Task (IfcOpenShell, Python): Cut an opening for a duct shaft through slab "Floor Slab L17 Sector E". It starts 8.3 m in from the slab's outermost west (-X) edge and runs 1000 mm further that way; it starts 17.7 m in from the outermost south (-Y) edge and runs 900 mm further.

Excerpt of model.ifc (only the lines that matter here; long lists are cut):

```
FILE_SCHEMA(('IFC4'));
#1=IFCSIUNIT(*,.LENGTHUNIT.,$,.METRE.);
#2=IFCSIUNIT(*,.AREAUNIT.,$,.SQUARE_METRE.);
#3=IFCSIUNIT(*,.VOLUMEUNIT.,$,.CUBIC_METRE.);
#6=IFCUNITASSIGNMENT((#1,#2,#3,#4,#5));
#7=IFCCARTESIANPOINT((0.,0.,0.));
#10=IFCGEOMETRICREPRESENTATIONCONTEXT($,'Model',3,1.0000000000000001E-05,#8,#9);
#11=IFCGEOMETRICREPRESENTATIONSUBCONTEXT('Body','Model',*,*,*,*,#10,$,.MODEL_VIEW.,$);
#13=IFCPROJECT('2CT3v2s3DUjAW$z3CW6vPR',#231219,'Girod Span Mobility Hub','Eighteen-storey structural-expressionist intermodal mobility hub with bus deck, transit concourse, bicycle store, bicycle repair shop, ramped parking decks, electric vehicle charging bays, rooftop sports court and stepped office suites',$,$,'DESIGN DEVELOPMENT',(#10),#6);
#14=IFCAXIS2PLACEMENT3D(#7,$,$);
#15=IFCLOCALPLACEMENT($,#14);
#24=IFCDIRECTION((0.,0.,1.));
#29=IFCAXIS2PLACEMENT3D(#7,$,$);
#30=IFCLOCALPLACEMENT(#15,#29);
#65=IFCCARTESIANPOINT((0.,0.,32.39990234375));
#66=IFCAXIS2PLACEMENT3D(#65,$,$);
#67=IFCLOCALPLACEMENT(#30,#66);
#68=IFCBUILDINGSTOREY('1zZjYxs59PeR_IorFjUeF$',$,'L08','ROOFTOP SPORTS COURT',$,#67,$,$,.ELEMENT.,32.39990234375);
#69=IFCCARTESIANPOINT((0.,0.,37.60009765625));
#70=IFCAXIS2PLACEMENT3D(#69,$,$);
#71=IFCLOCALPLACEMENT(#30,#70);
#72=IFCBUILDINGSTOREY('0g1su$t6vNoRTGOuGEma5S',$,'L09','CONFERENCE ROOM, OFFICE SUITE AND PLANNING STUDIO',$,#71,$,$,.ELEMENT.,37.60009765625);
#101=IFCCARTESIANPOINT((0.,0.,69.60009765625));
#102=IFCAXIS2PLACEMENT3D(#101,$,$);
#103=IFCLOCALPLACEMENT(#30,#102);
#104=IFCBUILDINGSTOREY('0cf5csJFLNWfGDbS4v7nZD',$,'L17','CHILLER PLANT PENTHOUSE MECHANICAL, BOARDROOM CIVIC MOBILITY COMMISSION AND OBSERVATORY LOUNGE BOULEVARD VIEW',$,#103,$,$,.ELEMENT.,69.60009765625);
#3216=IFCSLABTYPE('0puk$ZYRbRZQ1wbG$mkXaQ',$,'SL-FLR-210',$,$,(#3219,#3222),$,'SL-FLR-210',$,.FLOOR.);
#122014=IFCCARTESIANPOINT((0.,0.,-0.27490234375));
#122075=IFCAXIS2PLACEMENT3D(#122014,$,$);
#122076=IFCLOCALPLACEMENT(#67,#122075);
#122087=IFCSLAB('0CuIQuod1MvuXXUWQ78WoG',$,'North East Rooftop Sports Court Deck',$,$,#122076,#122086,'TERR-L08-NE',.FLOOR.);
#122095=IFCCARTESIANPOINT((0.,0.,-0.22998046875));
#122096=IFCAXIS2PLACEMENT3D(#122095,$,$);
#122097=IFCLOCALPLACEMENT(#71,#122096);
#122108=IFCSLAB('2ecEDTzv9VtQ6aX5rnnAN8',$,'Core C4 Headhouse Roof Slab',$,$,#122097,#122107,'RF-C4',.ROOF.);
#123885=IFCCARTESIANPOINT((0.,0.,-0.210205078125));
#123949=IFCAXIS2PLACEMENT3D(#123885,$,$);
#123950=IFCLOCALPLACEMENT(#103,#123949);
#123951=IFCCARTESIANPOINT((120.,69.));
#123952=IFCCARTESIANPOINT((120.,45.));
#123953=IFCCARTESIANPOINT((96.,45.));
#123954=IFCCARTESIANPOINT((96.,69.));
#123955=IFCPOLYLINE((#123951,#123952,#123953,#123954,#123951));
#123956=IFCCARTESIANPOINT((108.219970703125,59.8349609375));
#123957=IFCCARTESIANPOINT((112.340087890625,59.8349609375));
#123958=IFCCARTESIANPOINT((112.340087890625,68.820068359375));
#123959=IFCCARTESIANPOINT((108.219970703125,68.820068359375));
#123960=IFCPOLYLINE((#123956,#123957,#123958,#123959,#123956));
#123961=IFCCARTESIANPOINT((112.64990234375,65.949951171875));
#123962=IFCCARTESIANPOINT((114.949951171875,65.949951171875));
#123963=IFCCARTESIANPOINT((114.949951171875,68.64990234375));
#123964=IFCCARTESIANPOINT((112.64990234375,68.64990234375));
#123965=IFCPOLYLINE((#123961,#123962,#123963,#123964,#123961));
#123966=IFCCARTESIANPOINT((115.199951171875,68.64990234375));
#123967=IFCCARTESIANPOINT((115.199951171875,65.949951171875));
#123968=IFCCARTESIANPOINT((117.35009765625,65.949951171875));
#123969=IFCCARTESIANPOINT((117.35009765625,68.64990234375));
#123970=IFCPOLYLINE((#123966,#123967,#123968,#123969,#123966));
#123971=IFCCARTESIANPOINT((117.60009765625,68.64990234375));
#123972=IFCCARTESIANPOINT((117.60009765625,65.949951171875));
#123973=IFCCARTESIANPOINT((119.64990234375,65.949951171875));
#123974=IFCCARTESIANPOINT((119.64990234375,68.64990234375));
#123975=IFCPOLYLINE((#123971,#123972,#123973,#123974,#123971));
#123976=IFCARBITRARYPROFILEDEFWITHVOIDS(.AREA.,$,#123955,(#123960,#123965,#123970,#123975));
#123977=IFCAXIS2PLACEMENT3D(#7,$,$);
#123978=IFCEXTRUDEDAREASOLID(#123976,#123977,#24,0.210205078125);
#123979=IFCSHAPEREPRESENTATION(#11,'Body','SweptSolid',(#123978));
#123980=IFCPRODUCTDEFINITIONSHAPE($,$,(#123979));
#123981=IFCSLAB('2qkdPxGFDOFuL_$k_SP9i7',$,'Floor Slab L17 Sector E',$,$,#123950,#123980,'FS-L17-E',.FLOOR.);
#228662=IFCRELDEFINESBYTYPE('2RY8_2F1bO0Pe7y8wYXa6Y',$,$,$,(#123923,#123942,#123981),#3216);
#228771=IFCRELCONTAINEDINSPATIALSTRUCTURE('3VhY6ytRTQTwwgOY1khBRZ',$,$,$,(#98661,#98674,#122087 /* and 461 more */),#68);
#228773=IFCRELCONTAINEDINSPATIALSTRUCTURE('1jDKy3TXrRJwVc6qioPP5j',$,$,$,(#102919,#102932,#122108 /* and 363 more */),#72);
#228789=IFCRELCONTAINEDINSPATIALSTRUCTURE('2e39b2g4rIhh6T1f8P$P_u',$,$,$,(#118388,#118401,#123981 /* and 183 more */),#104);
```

```python
import numpy as np
import ifcopenshell
import ifcopenshell.api.feature
import ifcopenshell.api.geometry
import ifcopenshell.api.root
import ifcopenshell.geom
import ifcopenshell.util.placement
import ifcopenshell.util.representation
import ifcopenshell.util.shape
import ifcopenshell.util.unit

model = ifcopenshell.open("model.ifc")
unit_scale = ifcopenshell.util.unit.calculate_unit_scale(model)
settings = ifcopenshell.geom.settings()


def volume(element):
    """Net volume in cubic metres, openings subtracted."""
    shape = ifcopenshell.geom.create_shape(settings, element)
    return ifcopenshell.util.shape.get_volume(shape.geometry)


slab = model.by_guid("2qkdPxGFDOFuL_$k_SP9i7")
before = volume(slab)

# Extent in the slab's own axes, in metres. The edges named are its -X and -Y sides.
slab_shape = ifcopenshell.geom.create_shape(settings, slab)
vertices = ifcopenshell.util.shape.get_vertices(slab_shape.geometry)
x_min, y_min, bottom = vertices.min(axis=0)
top = vertices[:, 2].max()

opening = ifcopenshell.api.root.create_entity(model, ifc_class="IfcOpeningElement", name="Duct shaft opening", predefined_type="OPENING")
context = ifcopenshell.util.representation.get_context(model, "Model", "Body", "MODEL_VIEW")
width, depth = 1, 0.9
outline = [(0.0, 0.0), (width, 0.0), (width, depth), (0.0, depth), (0.0, 0.0)]
# Overshoot both faces by 50 mm so the cut is clean.
shape = ifcopenshell.api.geometry.add_slab_representation(
    model, context=context, depth=top - bottom + 0.1, polyline=outline
)
ifcopenshell.api.geometry.assign_representation(model, product=opening, representation=shape)

matrix = ifcopenshell.util.placement.get_local_placement(slab.ObjectPlacement)
matrix[:, 3] = matrix @ np.append(np.array([x_min + 8.3, y_min + 17.7, bottom - 0.05]) / unit_scale, 1.0)
ifcopenshell.api.geometry.edit_object_placement(model, product=opening, matrix=matrix, is_si=False)
ifcopenshell.api.feature.add_feature(model, feature=opening, element=slab)

after = volume(slab)

print(f"slab volume {before:.3f} -> {after:.3f} m3")

model.write("model_edited.ifc")
```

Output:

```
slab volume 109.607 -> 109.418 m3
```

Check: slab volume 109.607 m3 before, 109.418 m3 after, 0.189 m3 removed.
